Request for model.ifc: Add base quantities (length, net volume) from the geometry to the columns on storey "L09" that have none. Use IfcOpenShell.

First a look at what the model holds.

```python
import ifcopenshell
import ifcopenshell.util.element
import ifcopenshell.util.unit

model = ifcopenshell.open("model.ifc")
print(model.schema)
for unit_type in ("LENGTHUNIT", "AREAUNIT", "VOLUMEUNIT"):
    print(unit_type, ifcopenshell.util.unit.calculate_unit_scale(model, unit_type))
storey = next(s for s in model.by_type("IfcBuildingStorey") if s.Name == "L09")
columns = [e for e in ifcopenshell.util.element.get_decomposition(storey) if e.is_a("IfcColumn")]
for e in sorted(columns, key=lambda e: e.id()):
    print(e.id(), e.is_a(), e.Name, list(ifcopenshell.util.element.get_psets(e, qtos_only=True)), sep=" | ")
```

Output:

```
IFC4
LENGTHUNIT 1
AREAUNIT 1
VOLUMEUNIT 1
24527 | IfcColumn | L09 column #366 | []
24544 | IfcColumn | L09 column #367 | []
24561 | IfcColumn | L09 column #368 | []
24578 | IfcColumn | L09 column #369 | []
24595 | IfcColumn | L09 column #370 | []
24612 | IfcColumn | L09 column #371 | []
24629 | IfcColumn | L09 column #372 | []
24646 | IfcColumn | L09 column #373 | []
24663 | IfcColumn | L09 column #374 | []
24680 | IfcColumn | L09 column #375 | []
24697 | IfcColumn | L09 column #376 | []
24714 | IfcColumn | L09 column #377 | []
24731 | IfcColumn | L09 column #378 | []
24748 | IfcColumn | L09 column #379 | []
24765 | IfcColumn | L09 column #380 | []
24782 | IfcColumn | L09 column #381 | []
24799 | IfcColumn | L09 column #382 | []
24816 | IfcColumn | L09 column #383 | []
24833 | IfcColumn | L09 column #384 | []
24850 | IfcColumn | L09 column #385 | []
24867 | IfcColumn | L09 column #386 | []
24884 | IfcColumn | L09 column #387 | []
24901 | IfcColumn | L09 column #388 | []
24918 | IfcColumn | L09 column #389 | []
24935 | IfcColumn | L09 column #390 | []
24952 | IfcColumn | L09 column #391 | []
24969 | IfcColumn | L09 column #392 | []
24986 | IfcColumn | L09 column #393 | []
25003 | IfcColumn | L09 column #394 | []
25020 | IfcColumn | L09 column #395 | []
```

```python
import ifcopenshell
import ifcopenshell.api.pset
import ifcopenshell.geom
import ifcopenshell.util.element
import ifcopenshell.util.shape
import ifcopenshell.util.unit

model = ifcopenshell.open("model.ifc")
unit_scale = ifcopenshell.util.unit.calculate_unit_scale(model)
volume_scale = ifcopenshell.util.unit.calculate_unit_scale(model, "VOLUMEUNIT")
settings = ifcopenshell.geom.settings()

storey = next(s for s in model.by_type("IfcBuildingStorey") if s.Name == "L09")
columns = [e for e in ifcopenshell.util.element.get_decomposition(storey) if e.is_a("IfcColumn")]

for e in sorted(columns, key=lambda e: e.id()):
    if ifcopenshell.util.element.get_psets(e, qtos_only=True, should_inherit=False):
        continue
    # Geometry comes back in metres, in the element's own axes.
    shape = ifcopenshell.geom.create_shape(settings, e)
    values = {
        "Length": ifcopenshell.util.shape.get_z(shape.geometry) / unit_scale,
        "NetVolume": ifcopenshell.util.shape.get_volume(shape.geometry) / volume_scale,
    }
    qto = ifcopenshell.api.pset.add_qto(model, product=e, name="Qto_ColumnBaseQuantities")
    ifcopenshell.api.pset.edit_qto(model, qto=qto, properties=values)
    print(e.id(), {k: round(v, 3) for k, v in values.items()})

model.write("model_rev.ifc")
```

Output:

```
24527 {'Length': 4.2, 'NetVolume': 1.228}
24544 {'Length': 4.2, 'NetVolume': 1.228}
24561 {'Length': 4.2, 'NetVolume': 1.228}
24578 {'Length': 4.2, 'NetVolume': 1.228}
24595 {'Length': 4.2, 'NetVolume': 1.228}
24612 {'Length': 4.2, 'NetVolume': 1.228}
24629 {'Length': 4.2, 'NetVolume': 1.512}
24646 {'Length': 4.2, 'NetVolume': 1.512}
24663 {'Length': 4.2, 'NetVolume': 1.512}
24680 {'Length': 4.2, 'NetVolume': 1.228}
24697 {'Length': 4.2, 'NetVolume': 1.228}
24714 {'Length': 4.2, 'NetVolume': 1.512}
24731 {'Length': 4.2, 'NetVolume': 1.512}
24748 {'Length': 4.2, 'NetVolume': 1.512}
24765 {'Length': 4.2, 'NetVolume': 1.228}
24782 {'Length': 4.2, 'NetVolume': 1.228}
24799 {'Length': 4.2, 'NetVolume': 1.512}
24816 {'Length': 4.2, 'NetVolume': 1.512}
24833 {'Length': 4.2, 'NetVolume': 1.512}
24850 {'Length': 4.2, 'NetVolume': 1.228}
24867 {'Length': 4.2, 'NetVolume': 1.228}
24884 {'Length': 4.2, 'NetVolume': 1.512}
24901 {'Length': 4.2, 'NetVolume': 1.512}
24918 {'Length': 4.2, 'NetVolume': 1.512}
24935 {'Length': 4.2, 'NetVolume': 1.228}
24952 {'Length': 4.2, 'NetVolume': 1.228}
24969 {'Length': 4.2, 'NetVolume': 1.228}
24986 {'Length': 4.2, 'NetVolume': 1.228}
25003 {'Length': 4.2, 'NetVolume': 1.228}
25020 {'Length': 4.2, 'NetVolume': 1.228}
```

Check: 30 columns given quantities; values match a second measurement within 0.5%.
